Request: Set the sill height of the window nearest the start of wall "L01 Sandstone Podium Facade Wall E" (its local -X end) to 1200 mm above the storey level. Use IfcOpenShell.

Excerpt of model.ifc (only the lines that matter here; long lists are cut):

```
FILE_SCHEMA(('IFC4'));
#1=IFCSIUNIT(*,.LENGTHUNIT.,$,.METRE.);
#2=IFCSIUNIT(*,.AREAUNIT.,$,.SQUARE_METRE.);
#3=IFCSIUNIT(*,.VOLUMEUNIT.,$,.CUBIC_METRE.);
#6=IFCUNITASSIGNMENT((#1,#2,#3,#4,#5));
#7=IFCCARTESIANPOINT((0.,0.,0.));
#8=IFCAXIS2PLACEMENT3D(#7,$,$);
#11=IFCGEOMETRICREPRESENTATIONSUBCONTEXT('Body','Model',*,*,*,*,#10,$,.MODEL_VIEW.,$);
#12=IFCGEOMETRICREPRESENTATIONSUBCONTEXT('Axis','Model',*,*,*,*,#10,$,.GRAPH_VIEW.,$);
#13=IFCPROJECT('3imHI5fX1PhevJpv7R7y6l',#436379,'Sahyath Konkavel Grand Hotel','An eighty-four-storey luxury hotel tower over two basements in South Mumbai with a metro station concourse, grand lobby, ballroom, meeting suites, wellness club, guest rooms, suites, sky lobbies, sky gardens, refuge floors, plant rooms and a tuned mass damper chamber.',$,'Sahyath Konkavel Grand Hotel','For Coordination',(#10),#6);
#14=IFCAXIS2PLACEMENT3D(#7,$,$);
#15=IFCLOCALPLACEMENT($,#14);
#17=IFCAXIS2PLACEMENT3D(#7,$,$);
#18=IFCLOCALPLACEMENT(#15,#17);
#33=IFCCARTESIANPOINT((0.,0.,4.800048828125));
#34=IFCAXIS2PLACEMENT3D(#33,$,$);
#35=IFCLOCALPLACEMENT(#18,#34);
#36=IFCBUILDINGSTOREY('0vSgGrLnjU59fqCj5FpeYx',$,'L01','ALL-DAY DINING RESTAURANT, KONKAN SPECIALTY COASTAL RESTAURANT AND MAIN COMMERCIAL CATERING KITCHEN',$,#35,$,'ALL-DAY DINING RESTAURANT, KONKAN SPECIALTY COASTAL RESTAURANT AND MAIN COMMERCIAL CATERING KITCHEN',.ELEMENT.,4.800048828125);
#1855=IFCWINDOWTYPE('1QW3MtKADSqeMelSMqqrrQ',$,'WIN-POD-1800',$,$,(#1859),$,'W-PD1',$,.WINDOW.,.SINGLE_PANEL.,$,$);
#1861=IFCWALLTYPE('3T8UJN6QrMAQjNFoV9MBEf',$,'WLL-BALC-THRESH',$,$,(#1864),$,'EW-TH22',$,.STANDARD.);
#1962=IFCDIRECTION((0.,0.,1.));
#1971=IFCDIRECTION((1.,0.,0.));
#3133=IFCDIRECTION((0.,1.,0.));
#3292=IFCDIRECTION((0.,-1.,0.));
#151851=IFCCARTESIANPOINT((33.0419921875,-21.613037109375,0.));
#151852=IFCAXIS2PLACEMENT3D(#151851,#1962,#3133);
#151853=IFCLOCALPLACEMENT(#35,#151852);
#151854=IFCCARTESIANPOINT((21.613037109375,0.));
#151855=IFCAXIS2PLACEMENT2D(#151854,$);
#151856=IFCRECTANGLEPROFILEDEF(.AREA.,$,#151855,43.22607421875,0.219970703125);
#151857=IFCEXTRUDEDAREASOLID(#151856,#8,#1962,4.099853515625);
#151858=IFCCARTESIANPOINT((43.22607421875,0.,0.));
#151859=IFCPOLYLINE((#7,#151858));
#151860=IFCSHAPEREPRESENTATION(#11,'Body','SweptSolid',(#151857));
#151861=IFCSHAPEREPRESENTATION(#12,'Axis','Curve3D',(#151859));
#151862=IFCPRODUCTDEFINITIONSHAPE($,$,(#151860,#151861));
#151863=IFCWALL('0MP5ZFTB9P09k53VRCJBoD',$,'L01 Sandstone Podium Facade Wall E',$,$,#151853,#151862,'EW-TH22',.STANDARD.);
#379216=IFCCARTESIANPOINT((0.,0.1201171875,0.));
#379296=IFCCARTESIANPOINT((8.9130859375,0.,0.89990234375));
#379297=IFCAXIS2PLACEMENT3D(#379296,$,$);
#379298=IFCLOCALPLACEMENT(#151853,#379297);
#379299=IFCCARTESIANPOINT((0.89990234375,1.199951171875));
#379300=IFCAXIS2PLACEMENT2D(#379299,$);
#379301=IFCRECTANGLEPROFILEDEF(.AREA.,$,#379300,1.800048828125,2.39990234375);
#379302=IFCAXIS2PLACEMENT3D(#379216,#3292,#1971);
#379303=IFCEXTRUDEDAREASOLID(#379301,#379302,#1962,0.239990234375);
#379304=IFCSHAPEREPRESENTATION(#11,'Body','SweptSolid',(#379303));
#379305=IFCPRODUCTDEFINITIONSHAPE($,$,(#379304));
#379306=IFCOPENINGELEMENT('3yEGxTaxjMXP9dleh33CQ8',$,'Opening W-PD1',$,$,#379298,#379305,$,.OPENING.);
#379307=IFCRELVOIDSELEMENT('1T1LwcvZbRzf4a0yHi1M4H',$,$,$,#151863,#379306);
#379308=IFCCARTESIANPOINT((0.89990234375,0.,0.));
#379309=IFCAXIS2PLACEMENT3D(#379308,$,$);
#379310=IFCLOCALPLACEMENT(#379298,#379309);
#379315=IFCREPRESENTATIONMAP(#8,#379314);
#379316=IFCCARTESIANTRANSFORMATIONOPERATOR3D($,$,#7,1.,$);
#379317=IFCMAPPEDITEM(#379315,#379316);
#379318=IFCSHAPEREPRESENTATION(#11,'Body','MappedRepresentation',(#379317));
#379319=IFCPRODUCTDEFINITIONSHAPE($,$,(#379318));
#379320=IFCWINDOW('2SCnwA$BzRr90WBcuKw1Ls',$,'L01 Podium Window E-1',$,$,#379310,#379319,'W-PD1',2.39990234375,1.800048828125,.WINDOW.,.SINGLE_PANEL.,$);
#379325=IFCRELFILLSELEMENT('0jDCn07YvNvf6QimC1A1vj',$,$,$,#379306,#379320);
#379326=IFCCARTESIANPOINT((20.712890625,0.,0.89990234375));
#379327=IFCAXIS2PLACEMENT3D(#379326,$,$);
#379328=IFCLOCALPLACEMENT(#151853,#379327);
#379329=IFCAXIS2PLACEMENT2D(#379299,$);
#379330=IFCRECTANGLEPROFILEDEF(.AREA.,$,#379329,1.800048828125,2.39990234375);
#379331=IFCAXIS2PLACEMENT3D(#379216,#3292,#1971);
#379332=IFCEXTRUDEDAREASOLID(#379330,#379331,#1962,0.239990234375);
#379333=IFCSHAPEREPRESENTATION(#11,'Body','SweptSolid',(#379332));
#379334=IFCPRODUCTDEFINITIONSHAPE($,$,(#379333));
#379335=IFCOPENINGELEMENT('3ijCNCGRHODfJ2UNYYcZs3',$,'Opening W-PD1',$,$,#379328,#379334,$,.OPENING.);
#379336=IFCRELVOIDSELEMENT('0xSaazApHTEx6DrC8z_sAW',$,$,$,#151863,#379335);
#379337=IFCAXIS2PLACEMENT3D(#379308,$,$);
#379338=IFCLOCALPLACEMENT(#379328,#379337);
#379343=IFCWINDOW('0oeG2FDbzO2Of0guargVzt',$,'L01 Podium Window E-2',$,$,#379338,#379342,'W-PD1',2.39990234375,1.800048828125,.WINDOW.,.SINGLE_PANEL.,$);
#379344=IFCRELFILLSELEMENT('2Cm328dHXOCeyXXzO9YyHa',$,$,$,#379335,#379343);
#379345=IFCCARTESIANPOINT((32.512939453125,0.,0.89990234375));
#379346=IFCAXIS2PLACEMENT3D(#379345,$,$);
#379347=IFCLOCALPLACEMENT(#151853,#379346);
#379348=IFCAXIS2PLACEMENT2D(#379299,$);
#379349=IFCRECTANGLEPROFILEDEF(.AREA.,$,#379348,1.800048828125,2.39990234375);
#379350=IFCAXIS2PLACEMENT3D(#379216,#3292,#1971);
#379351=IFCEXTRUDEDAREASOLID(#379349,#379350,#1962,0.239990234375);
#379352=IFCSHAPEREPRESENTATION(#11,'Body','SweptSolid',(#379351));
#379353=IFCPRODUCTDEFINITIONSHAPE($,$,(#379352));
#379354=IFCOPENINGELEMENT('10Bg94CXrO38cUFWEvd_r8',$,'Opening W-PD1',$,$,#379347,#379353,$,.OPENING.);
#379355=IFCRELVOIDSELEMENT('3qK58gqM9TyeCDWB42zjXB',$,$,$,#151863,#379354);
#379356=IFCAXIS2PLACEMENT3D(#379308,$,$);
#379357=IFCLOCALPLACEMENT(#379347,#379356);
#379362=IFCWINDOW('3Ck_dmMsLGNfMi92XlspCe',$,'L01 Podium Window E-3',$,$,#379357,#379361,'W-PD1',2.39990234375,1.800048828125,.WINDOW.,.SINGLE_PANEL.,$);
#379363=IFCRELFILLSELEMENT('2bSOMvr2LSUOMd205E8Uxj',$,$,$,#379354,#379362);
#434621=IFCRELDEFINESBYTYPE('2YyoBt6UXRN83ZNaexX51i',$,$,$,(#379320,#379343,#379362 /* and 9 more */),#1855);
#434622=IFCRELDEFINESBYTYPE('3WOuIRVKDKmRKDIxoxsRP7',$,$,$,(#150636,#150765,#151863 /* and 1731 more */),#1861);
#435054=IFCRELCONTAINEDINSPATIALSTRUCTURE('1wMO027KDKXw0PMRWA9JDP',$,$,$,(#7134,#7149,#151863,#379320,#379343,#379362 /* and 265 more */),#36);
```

```python
import numpy as np
import ifcopenshell
import ifcopenshell.api.geometry
import ifcopenshell.geom
import ifcopenshell.util.element
import ifcopenshell.util.placement
import ifcopenshell.util.shape
import ifcopenshell.util.unit

model = ifcopenshell.open("model.ifc")
unit_scale = ifcopenshell.util.unit.calculate_unit_scale(model)

window = model.by_guid("2SCnwA$BzRr90WBcuKw1Ls")
opening = window.FillsVoids[0].RelatingOpeningElement
storey = ifcopenshell.util.element.get_container(window, ifc_class="IfcBuildingStorey")
level = ifcopenshell.util.placement.get_local_placement(storey.ObjectPlacement)[2, 3]

# The opening's origin need not be at the sill, so measure its lowest point.
shape = ifcopenshell.geom.create_shape(ifcopenshell.geom.settings(), opening)
bottom = ifcopenshell.util.shape.get_shape_bottom_elevation(shape, shape.geometry) / unit_scale
dz = level + 1.2 - bottom

shift = np.array([0.0, 0.0, dz])
# The window is placed relative to its opening, so it follows when the opening moves.
matrix = ifcopenshell.util.placement.get_local_placement(opening.ObjectPlacement)
matrix[:3, 3] += shift
ifcopenshell.api.geometry.edit_object_placement(
    model, product=opening, matrix=matrix, is_si=False, should_transform_children=True
)

print(f"moved by {dz * unit_scale:+.3f} m")

model.write("model_updated.ifc")
```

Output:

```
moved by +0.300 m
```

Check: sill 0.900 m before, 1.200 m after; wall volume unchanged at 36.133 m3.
